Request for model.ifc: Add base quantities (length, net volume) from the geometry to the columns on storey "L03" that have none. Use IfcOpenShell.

First a look at what the model holds.

```python
import ifcopenshell
import ifcopenshell.util.element
import ifcopenshell.util.unit

model = ifcopenshell.open("model.ifc")
print(model.schema)
for unit_type in ("LENGTHUNIT", "AREAUNIT", "VOLUMEUNIT"):
    print(unit_type, ifcopenshell.util.unit.calculate_unit_scale(model, unit_type))
storey = next(s for s in model.by_type("IfcBuildingStorey") if s.Name == "L03")
columns = [e for e in ifcopenshell.util.element.get_decomposition(storey) if e.is_a("IfcColumn")]
for e in sorted(columns, key=lambda e: e.id()):
    print(e.id(), e.is_a(), e.Name, list(ifcopenshell.util.element.get_psets(e, qtos_only=True)), sep=" | ")
```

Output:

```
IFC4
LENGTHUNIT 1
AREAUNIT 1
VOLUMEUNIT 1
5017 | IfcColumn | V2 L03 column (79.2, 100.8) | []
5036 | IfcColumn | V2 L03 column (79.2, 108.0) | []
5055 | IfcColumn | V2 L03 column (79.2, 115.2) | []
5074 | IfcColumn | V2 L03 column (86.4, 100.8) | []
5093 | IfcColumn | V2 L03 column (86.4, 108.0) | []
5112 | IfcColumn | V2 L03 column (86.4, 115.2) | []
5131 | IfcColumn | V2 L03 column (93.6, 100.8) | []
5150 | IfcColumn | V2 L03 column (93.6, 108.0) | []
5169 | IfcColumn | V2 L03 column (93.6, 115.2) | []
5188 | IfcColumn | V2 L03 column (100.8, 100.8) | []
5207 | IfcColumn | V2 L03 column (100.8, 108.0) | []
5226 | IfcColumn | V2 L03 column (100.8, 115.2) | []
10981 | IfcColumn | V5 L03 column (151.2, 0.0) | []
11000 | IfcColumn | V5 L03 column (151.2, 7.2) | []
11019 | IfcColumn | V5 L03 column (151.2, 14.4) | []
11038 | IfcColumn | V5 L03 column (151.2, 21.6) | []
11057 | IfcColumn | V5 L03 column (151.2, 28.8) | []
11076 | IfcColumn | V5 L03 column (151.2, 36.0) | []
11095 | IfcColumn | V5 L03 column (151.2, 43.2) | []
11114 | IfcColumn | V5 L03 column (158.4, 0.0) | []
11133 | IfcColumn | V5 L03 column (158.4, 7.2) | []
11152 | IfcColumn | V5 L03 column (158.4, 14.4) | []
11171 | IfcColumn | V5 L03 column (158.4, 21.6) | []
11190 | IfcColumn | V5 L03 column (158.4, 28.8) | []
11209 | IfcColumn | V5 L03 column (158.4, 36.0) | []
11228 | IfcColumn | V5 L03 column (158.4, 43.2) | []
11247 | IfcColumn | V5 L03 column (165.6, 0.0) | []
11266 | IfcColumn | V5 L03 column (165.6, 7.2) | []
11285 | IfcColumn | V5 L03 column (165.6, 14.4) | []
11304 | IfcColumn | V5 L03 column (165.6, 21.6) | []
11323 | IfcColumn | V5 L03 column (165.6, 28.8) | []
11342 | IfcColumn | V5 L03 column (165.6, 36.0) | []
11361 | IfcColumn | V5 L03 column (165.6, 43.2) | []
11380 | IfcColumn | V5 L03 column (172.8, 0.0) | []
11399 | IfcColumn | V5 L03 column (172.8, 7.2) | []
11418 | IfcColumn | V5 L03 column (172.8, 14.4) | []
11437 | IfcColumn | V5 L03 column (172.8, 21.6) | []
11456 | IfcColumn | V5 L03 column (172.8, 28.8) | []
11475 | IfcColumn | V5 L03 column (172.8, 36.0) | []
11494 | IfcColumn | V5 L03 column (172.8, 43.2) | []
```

```python
import ifcopenshell
import ifcopenshell.api.pset
import ifcopenshell.geom
import ifcopenshell.util.element
import ifcopenshell.util.shape
import ifcopenshell.util.unit

model = ifcopenshell.open("model.ifc")
unit_scale = ifcopenshell.util.unit.calculate_unit_scale(model)
volume_scale = ifcopenshell.util.unit.calculate_unit_scale(model, "VOLUMEUNIT")
settings = ifcopenshell.geom.settings()

storey = next(s for s in model.by_type("IfcBuildingStorey") if s.Name == "L03")
columns = [e for e in ifcopenshell.util.element.get_decomposition(storey) if e.is_a("IfcColumn")]

for e in sorted(columns, key=lambda e: e.id()):
    if ifcopenshell.util.element.get_psets(e, qtos_only=True, should_inherit=False):
        continue
    # Geometry comes back in metres, in the element's own axes.
    shape = ifcopenshell.geom.create_shape(settings, e)
    values = {
        "Length": ifcopenshell.util.shape.get_z(shape.geometry) / unit_scale,
        "NetVolume": ifcopenshell.util.shape.get_volume(shape.geometry) / volume_scale,
    }
    qto = ifcopenshell.api.pset.add_qto(model, product=e, name="Qto_ColumnBaseQuantities")
    ifcopenshell.api.pset.edit_qto(model, qto=qto, properties=values)
    print(e.id(), {k: round(v, 3) for k, v in values.items()})

model.write("model-out.ifc")
```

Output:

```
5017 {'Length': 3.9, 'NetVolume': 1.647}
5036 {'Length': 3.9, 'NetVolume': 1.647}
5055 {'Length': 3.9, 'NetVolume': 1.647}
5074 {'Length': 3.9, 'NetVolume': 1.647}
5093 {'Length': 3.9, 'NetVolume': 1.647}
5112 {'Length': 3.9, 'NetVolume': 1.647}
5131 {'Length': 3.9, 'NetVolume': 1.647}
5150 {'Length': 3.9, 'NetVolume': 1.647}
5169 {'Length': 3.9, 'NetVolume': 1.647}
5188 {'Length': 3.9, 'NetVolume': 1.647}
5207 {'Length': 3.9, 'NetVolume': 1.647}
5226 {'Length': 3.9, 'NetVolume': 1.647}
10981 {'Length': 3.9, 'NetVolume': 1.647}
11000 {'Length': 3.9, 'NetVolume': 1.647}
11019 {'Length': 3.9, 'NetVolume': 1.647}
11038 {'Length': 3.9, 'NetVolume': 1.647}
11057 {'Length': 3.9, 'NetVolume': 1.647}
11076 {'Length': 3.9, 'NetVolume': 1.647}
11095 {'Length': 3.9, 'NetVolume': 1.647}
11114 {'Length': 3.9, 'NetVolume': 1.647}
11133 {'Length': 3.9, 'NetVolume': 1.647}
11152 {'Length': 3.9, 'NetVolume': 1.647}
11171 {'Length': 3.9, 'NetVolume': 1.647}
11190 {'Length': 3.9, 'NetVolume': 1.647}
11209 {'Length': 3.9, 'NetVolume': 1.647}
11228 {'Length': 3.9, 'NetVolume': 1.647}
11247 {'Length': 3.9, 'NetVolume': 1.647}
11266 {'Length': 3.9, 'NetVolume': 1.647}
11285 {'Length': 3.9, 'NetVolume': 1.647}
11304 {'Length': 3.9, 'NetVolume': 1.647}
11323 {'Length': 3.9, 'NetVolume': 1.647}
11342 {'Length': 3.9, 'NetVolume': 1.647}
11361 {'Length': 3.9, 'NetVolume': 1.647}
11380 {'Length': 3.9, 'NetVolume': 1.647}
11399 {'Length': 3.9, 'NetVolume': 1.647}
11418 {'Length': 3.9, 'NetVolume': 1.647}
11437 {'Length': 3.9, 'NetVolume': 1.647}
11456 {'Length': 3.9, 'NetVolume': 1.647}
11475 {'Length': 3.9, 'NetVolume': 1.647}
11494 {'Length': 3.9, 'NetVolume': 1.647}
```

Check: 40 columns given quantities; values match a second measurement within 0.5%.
